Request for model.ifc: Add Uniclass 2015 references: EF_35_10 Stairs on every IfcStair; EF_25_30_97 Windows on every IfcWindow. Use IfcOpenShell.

First a look at what the model holds.

```python
import ifcopenshell

model = ifcopenshell.open("model.ifc")
print(model.schema)
print("classifications:", [c.Name for c in model.by_type("IfcClassification")])
for ifc_class in ("IfcDoor", "IfcRoof", "IfcStair", "IfcWall", "IfcWindow"):
    print(ifc_class, len(model.by_type(ifc_class)))
```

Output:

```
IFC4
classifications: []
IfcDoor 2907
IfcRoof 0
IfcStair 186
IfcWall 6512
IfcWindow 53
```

```python
import ifcopenshell
import ifcopenshell.api.classification

model = ifcopenshell.open("model.ifc")

system = ifcopenshell.api.classification.add_classification(model, classification="Uniclass 2015")

codes = {
    "IfcStair": ("EF_35_10", "Stairs"),
    "IfcWindow": ("EF_25_30_97", "Windows"),
}
for ifc_class, (code, name) in codes.items():
    products = model.by_type(ifc_class)
    ifcopenshell.api.classification.add_reference(
        model, products=products, classification=system, identification=code, name=name
    )
    print(code, len(products))

model.write("model_rev.ifc")
```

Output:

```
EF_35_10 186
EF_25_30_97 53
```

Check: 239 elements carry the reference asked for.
